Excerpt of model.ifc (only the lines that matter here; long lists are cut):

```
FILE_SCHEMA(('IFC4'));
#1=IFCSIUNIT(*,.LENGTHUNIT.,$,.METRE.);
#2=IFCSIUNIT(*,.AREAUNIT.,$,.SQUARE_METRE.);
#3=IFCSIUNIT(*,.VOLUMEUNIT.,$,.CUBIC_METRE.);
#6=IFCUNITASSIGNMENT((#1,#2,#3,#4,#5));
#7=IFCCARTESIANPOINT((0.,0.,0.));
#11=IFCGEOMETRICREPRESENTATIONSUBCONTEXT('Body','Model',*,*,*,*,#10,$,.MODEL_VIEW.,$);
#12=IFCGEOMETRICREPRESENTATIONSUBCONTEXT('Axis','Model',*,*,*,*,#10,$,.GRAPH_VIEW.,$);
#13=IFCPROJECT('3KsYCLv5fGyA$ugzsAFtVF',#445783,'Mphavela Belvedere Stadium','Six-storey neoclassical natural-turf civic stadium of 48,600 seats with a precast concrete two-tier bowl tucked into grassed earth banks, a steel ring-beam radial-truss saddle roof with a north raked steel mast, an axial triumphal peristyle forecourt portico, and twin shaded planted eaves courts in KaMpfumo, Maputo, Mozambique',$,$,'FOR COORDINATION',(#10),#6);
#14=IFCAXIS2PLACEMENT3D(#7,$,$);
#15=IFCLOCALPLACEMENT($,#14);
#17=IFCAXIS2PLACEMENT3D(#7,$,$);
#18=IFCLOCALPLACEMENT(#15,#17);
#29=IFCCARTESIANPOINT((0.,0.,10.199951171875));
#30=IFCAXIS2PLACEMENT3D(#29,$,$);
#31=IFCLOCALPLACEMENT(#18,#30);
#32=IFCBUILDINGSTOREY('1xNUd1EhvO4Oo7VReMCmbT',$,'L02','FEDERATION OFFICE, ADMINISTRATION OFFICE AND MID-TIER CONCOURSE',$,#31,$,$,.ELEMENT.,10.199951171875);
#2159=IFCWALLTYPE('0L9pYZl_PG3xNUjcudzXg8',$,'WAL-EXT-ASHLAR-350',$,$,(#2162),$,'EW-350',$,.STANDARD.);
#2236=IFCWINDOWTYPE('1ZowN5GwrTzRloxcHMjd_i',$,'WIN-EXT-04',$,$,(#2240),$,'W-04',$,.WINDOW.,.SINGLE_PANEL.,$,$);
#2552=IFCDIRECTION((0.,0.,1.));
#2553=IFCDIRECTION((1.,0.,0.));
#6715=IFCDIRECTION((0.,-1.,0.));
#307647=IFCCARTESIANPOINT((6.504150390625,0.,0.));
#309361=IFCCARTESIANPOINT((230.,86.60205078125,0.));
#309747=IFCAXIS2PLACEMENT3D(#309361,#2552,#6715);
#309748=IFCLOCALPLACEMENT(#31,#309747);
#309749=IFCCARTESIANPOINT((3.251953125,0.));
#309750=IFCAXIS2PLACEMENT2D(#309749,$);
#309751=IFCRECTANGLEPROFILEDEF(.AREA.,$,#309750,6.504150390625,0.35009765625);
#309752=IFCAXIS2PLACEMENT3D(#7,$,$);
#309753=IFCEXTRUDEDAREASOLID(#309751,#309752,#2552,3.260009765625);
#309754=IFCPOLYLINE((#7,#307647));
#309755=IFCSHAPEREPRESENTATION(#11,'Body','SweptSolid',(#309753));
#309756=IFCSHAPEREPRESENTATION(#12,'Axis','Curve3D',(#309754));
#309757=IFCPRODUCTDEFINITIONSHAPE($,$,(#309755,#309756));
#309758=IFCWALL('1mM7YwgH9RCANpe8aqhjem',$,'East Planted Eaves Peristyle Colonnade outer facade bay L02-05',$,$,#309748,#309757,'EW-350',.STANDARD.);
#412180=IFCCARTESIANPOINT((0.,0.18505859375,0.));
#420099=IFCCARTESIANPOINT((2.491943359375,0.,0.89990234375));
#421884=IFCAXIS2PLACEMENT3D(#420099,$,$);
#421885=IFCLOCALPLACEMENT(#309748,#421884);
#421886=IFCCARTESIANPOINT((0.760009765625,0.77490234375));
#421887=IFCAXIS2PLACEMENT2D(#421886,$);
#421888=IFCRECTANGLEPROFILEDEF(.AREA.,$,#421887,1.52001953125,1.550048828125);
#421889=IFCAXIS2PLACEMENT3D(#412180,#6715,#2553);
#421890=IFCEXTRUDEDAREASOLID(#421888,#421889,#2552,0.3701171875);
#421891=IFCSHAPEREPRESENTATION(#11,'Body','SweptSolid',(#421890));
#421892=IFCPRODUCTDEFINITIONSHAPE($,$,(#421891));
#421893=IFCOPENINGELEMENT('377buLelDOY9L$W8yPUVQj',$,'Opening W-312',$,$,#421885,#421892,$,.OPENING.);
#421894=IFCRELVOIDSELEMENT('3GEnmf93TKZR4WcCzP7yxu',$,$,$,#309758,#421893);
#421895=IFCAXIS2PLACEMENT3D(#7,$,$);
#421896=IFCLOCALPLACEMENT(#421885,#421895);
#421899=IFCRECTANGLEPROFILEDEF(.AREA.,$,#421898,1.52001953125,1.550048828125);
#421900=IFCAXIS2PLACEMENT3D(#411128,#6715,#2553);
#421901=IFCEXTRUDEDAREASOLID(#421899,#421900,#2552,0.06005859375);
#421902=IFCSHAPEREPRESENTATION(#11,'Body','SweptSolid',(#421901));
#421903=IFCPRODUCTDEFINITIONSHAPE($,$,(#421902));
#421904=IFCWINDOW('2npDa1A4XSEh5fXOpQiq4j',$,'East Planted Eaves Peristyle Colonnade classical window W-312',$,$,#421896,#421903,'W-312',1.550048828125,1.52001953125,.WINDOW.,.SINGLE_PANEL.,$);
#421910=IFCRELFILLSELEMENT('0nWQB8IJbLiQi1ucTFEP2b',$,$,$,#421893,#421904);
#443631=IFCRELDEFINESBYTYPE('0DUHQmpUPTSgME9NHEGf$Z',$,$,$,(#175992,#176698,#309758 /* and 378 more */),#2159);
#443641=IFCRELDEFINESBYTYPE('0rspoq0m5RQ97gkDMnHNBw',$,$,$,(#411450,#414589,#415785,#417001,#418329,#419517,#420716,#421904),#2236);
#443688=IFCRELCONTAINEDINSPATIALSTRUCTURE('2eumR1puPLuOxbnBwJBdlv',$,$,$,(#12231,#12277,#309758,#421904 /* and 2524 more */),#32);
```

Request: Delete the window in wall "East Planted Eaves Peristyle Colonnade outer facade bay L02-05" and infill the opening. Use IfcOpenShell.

```python
import ifcopenshell
import ifcopenshell.api.feature
import ifcopenshell.api.root
import ifcopenshell.geom
import ifcopenshell.util.shape

model = ifcopenshell.open("model.ifc")
settings = ifcopenshell.geom.settings()


def volume(element):
    """Net volume in cubic metres, openings subtracted."""
    shape = ifcopenshell.geom.create_shape(settings, element)
    return ifcopenshell.util.shape.get_volume(shape.geometry)


window = model.by_guid("2npDa1A4XSEh5fXOpQiq4j")
opening = window.FillsVoids[0].RelatingOpeningElement
wall = opening.VoidsElements[0].RelatingBuildingElement
before = volume(wall)

ifcopenshell.api.root.remove_product(model, product=window)
ifcopenshell.api.feature.remove_feature(model, feature=opening)

after = volume(wall)

print(f"wall volume {before:.3f} -> {after:.3f} m3")

model.write("model_updated.ifc")
```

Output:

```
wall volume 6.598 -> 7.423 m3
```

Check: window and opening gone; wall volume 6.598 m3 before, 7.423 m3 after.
